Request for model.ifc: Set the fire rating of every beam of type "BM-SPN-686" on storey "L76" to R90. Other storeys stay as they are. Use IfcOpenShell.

First a look at what the model holds.

```python
import ifcopenshell
import ifcopenshell.util.element

model = ifcopenshell.open("model.ifc")
print(model.schema)
storey = next(s for s in model.by_type("IfcBuildingStorey") if s.Name == "L76")
beams = [e for e in ifcopenshell.util.element.get_decomposition(storey) if e.is_a("IfcBeam")]
seen = {}
for e in beams:
    element_type = ifcopenshell.util.element.get_type(e)
    key = (element_type.Name if element_type != e and element_type else None, ifcopenshell.util.element.get_pset(e, "Pset_BeamCommon", "FireRating"))
    seen[key] = seen.get(key, 0) + 1
for (name, value), count in sorted(seen.items(), key=str):
    print(count, "x", name, "|", value)
```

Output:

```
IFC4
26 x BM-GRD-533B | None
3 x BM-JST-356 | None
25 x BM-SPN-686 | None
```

```python
import ifcopenshell
import ifcopenshell.api.pset
import ifcopenshell.util.element

model = ifcopenshell.open("model.ifc")

storey = next(s for s in model.by_type("IfcBuildingStorey") if s.Name == "L76")
beams = [e for e in ifcopenshell.util.element.get_decomposition(storey) if e.is_a("IfcBeam")]

count = 0
for e in beams:
    element_type = ifcopenshell.util.element.get_type(e)
    if element_type in (None, e) or element_type.Name != "BM-SPN-686":
        continue
    found = ifcopenshell.util.element.get_pset(e, "Pset_BeamCommon", should_inherit=False)
    if found:
        pset = model.by_id(found["id"])
        if len(ifcopenshell.util.element.get_elements_by_pset(pset)) > 1:
            pset = ifcopenshell.api.pset.unshare_pset(model, products=[e], pset=pset)[0]
    else:
        pset = ifcopenshell.api.pset.add_pset(model, product=e, name="Pset_BeamCommon")
    ifcopenshell.api.pset.edit_pset(model, pset=pset, properties={"FireRating": "R90"})
    count += 1

print(count, "beams updated")

model.write("model_rev.ifc")
```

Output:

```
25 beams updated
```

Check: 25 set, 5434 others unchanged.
